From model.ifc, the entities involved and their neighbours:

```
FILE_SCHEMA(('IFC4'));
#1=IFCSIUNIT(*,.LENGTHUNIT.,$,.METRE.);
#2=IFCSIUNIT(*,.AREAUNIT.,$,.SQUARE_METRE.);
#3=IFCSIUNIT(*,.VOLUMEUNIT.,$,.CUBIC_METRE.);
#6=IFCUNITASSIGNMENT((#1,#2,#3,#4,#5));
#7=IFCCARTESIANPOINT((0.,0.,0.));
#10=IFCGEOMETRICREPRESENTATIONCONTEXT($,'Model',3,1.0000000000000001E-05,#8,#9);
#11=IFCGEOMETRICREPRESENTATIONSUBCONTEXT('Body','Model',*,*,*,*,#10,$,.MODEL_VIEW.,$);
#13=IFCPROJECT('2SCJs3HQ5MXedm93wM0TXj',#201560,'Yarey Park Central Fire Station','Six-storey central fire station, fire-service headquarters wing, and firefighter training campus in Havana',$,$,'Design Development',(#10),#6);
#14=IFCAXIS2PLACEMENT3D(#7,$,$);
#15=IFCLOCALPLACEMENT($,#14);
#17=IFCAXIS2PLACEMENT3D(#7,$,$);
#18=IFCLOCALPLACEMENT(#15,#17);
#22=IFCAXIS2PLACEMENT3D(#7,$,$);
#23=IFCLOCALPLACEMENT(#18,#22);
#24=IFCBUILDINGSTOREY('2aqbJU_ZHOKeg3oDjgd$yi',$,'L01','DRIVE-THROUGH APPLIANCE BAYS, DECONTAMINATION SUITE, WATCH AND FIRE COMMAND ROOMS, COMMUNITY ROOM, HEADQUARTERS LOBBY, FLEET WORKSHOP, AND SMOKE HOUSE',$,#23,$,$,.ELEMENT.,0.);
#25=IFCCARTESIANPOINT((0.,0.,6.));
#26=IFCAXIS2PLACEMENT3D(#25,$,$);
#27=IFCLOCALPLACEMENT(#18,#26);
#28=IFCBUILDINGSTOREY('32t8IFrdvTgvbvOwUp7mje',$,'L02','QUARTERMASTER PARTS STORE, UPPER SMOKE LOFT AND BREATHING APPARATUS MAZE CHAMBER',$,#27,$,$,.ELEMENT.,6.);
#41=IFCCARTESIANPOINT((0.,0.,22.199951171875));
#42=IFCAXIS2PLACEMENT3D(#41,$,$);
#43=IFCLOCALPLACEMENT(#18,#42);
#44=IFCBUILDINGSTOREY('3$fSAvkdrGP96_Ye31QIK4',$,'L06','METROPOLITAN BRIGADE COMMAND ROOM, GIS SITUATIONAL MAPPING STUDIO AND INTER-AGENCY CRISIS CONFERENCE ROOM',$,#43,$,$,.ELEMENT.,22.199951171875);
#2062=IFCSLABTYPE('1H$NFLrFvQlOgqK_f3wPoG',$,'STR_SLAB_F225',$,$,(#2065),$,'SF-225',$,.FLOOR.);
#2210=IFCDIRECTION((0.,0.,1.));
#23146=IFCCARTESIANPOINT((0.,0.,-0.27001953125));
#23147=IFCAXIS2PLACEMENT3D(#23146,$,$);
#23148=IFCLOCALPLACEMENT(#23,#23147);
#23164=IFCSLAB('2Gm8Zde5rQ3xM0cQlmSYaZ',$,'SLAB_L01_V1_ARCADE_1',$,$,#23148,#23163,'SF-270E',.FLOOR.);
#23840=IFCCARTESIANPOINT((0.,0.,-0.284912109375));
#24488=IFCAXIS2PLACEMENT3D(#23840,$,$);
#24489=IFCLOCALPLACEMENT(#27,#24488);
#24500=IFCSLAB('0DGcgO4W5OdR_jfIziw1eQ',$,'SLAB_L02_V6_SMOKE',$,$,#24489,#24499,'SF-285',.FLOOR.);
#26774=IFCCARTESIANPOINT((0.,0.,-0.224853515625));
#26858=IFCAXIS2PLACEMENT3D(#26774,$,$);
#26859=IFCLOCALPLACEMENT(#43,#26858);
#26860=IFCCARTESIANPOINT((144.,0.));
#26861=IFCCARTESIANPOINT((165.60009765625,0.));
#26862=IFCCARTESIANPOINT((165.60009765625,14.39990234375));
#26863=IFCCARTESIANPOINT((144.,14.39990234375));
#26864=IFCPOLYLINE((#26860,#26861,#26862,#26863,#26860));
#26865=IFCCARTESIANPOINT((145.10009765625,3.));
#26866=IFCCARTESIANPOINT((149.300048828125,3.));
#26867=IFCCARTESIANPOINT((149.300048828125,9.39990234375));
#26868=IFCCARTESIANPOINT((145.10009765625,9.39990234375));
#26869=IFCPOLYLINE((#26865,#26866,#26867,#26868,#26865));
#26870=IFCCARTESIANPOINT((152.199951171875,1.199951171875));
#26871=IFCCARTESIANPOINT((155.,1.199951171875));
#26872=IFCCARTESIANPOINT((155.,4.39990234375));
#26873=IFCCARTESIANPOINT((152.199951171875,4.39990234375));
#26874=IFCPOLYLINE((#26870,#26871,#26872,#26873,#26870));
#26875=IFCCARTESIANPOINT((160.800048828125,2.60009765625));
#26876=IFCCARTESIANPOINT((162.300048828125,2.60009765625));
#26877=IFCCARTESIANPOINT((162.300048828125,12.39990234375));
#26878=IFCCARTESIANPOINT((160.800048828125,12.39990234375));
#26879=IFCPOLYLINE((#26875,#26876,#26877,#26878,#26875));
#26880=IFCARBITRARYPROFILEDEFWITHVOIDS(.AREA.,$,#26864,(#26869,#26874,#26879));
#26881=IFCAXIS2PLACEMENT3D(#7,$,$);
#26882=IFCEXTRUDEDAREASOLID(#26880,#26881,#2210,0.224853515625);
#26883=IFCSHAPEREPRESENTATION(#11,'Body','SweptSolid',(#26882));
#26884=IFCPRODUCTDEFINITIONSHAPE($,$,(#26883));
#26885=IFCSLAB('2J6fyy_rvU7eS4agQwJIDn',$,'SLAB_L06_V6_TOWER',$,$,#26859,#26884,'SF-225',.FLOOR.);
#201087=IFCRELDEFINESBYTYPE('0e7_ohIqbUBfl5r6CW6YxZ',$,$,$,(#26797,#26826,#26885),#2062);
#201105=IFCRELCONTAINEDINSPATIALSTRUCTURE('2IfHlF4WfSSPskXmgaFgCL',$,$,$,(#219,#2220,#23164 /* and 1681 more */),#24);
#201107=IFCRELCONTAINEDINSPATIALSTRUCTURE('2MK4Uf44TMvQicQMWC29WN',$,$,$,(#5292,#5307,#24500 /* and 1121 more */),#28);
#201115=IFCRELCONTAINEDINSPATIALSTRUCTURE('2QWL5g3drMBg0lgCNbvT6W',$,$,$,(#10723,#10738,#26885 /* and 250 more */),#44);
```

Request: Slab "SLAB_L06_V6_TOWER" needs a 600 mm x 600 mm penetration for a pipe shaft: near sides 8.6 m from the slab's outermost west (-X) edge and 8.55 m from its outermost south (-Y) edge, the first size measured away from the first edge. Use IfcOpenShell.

```python
import numpy as np
import ifcopenshell
import ifcopenshell.api.feature
import ifcopenshell.api.geometry
import ifcopenshell.api.root
import ifcopenshell.geom
import ifcopenshell.util.placement
import ifcopenshell.util.representation
import ifcopenshell.util.shape
import ifcopenshell.util.unit

model = ifcopenshell.open("model.ifc")
unit_scale = ifcopenshell.util.unit.calculate_unit_scale(model)
settings = ifcopenshell.geom.settings()


def volume(element):
    """Net volume in cubic metres, openings subtracted."""
    shape = ifcopenshell.geom.create_shape(settings, element)
    return ifcopenshell.util.shape.get_volume(shape.geometry)


slab = model.by_guid("2J6fyy_rvU7eS4agQwJIDn")
before = volume(slab)

# Extent in the slab's own axes, in metres. The edges named are its -X and -Y sides.
slab_shape = ifcopenshell.geom.create_shape(settings, slab)
vertices = ifcopenshell.util.shape.get_vertices(slab_shape.geometry)
x_min, y_min, bottom = vertices.min(axis=0)
top = vertices[:, 2].max()

opening = ifcopenshell.api.root.create_entity(model, ifc_class="IfcOpeningElement", name="Pipe shaft opening", predefined_type="OPENING")
context = ifcopenshell.util.representation.get_context(model, "Model", "Body", "MODEL_VIEW")
width, depth = 0.6, 0.6
outline = [(0.0, 0.0), (width, 0.0), (width, depth), (0.0, depth), (0.0, 0.0)]
# Overshoot both faces by 50 mm so the cut is clean.
shape = ifcopenshell.api.geometry.add_slab_representation(
    model, context=context, depth=top - bottom + 0.1, polyline=outline
)
ifcopenshell.api.geometry.assign_representation(model, product=opening, representation=shape)

matrix = ifcopenshell.util.placement.get_local_placement(slab.ObjectPlacement)
matrix[:, 3] = matrix @ np.append(np.array([x_min + 8.6, y_min + 8.55, bottom - 0.05]) / unit_scale, 1.0)
ifcopenshell.api.geometry.edit_object_placement(model, product=opening, matrix=matrix, is_si=False)
ifcopenshell.api.feature.add_feature(model, feature=opening, element=slab)

after = volume(slab)

print(f"slab volume {before:.3f} -> {after:.3f} m3")

model.write("model_edited.ifc")
```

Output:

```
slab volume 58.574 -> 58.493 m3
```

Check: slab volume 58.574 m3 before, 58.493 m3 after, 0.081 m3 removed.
